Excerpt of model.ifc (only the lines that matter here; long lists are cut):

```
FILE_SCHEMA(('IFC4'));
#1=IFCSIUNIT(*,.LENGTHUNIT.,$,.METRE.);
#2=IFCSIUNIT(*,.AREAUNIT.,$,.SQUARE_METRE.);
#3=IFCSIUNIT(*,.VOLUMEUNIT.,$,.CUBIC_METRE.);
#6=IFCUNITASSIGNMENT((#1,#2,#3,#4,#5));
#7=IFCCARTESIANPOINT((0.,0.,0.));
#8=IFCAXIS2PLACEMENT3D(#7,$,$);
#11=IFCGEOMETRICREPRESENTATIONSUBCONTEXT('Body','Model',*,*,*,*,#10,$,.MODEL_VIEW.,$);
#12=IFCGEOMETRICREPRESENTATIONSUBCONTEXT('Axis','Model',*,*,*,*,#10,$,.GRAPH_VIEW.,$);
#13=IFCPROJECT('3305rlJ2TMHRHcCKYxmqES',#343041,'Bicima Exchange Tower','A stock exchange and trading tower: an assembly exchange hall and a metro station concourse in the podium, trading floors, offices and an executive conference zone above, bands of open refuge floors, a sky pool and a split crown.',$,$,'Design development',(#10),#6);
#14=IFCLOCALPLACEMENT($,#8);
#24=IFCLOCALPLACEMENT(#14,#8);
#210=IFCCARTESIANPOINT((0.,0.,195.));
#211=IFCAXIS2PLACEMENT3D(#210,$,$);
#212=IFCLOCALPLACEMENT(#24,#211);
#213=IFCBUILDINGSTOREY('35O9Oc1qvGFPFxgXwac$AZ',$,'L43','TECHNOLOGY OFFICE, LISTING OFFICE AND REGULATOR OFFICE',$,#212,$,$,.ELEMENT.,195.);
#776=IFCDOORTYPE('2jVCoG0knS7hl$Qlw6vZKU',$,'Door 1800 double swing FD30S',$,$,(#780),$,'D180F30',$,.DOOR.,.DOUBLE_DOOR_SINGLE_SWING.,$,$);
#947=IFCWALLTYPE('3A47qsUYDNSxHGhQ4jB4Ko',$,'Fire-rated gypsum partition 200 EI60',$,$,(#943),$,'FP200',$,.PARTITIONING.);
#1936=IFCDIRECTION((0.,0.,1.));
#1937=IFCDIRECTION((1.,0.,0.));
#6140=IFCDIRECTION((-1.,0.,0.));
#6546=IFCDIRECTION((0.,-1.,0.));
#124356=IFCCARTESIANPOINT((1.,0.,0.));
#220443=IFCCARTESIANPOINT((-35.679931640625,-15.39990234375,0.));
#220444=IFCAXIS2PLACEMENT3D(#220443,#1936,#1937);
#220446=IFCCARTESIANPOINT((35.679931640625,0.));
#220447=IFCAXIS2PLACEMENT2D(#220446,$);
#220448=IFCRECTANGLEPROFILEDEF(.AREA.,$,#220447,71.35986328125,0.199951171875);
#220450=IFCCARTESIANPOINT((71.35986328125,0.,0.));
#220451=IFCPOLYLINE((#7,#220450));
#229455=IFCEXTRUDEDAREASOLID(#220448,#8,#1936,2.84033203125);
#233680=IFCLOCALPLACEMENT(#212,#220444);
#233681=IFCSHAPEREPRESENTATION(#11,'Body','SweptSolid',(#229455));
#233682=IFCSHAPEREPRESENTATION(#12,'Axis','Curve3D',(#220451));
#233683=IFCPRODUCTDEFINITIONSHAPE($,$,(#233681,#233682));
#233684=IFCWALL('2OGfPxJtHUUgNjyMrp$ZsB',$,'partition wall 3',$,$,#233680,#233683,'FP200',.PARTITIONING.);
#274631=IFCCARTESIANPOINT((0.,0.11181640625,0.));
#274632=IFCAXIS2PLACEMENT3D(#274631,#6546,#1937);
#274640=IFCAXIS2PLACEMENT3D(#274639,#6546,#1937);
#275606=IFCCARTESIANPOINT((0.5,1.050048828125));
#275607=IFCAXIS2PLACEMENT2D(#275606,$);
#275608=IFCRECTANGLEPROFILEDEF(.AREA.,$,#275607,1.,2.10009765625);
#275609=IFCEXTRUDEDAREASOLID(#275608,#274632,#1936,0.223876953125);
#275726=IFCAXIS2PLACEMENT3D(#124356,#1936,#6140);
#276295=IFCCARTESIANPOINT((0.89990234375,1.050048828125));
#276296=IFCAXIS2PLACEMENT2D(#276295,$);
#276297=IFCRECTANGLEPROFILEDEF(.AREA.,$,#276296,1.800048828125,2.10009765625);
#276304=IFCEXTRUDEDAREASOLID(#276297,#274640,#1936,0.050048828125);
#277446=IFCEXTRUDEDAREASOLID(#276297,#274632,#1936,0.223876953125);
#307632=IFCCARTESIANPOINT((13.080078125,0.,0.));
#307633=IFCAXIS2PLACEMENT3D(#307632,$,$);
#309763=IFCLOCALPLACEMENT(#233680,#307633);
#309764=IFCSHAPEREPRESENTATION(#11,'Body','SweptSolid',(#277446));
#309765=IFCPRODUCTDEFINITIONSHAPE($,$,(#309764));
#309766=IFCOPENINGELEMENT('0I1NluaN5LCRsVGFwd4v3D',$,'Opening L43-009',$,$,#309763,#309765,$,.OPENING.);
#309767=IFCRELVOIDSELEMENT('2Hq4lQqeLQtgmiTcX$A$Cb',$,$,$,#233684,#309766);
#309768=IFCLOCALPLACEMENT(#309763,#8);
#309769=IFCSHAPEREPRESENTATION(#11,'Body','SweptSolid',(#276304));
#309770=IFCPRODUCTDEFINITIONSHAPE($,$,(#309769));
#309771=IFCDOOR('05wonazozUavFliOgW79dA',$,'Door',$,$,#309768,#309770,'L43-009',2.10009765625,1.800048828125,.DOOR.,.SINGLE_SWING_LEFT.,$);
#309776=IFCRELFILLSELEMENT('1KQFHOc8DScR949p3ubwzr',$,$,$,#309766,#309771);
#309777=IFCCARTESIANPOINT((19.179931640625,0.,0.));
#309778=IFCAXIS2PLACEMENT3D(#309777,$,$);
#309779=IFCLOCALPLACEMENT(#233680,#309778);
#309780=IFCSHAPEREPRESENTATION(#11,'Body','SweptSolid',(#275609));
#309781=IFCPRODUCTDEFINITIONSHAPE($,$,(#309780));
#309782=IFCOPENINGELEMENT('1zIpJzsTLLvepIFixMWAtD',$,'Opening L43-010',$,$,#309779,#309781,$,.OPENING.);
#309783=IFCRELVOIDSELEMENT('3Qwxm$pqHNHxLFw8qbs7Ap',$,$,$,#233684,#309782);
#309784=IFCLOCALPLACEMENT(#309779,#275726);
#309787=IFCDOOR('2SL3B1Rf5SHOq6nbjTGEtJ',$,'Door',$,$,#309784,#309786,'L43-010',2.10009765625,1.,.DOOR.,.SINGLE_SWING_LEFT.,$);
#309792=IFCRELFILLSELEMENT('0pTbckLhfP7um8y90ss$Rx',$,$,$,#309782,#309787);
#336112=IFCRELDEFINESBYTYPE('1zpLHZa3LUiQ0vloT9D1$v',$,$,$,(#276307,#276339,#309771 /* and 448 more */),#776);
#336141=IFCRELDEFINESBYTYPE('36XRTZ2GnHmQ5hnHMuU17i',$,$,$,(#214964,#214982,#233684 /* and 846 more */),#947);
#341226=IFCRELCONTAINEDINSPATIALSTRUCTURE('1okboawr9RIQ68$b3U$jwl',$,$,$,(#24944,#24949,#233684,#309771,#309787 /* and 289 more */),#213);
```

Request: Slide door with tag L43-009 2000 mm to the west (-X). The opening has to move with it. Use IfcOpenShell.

```python
import ifcopenshell
import ifcopenshell.api.geometry
import ifcopenshell.util.placement
import ifcopenshell.util.unit

model = ifcopenshell.open("model.ifc")
unit_scale = ifcopenshell.util.unit.calculate_unit_scale(model)

door = model.by_guid("05wonazozUavFliOgW79dA")
opening = door.FillsVoids[0].RelatingOpeningElement
wall = opening.VoidsElements[0].RelatingBuildingElement

wall_matrix = ifcopenshell.util.placement.get_local_placement(wall.ObjectPlacement)
shift = wall_matrix[:3, 0] * -2 / unit_scale
before = ifcopenshell.util.placement.get_local_placement(door.ObjectPlacement)[:3, 3].copy()

# The door is placed relative to its opening, so it follows when the opening moves.
matrix = ifcopenshell.util.placement.get_local_placement(opening.ObjectPlacement)
matrix[:3, 3] += shift
ifcopenshell.api.geometry.edit_object_placement(
    model, product=opening, matrix=matrix, is_si=False, should_transform_children=True
)

after = ifcopenshell.util.placement.get_local_placement(door.ObjectPlacement)[:3, 3]
print("door moved by", (after - before).round(3) + 0.0)

model.write("model_v2.ifc")
```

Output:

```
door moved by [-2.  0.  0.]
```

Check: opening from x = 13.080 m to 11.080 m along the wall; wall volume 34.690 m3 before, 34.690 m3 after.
